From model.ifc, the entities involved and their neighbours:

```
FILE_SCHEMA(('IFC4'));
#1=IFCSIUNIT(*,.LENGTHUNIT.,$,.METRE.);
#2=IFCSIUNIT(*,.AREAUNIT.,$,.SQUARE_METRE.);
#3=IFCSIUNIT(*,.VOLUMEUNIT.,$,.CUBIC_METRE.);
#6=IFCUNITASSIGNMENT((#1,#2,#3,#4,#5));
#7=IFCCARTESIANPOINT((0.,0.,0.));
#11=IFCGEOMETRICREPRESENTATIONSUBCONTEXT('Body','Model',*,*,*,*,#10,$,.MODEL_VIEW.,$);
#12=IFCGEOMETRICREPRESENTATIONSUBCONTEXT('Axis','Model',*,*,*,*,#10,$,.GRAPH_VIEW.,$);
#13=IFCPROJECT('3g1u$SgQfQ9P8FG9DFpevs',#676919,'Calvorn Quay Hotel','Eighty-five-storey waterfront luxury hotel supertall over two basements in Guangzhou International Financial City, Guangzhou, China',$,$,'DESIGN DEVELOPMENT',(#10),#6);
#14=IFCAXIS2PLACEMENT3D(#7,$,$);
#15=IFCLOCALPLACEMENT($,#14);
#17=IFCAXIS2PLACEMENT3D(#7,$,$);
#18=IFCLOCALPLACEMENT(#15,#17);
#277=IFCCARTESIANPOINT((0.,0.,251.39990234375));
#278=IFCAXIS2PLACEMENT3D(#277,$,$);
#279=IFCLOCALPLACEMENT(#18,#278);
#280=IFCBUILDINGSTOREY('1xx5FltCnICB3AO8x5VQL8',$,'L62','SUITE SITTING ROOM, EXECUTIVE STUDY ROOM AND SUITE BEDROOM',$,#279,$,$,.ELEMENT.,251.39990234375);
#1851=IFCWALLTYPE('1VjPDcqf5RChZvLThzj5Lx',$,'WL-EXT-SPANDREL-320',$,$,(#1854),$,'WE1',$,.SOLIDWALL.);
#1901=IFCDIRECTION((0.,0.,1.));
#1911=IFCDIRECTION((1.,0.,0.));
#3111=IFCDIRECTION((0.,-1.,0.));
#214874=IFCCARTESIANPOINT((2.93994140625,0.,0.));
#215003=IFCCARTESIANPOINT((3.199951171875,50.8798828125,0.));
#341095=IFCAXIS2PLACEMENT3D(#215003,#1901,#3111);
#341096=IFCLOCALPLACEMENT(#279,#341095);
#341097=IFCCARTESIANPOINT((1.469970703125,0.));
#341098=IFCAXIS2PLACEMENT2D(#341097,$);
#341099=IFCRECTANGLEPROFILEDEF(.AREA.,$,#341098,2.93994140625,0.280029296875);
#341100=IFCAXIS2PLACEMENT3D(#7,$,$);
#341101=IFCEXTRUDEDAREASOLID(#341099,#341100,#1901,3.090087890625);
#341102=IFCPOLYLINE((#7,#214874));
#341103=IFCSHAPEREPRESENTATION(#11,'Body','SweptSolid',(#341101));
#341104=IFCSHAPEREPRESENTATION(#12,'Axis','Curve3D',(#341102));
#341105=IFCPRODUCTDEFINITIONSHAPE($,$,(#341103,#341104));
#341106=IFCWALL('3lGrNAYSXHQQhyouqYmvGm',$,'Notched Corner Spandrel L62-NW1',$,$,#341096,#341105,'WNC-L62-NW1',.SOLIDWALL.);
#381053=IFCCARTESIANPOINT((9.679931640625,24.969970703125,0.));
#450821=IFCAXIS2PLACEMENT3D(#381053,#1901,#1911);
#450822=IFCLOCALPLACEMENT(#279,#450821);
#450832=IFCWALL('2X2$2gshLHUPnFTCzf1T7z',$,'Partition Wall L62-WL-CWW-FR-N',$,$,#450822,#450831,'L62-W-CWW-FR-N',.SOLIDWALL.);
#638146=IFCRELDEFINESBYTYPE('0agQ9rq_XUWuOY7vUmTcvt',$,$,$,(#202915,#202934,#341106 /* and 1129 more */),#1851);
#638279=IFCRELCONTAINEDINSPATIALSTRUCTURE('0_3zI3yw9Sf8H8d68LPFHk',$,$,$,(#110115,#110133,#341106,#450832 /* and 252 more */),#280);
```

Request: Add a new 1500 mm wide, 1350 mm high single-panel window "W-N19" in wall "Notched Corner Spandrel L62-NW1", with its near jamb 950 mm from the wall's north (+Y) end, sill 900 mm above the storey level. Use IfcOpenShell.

```python
import numpy as np
import ifcopenshell
import ifcopenshell.api.feature
import ifcopenshell.api.geometry
import ifcopenshell.api.root
import ifcopenshell.api.spatial
import ifcopenshell.geom
import ifcopenshell.util.element
import ifcopenshell.util.placement
import ifcopenshell.util.representation
import ifcopenshell.util.shape
import ifcopenshell.util.unit

model = ifcopenshell.open("model.ifc")
unit_scale = ifcopenshell.util.unit.calculate_unit_scale(model)
settings = ifcopenshell.geom.settings()


def volume(element):
    """Net volume in cubic metres, openings subtracted."""
    shape = ifcopenshell.geom.create_shape(settings, element)
    return ifcopenshell.util.shape.get_volume(shape.geometry)


wall = model.by_guid("3lGrNAYSXHQQhyouqYmvGm")
storey = ifcopenshell.util.element.get_container(wall, ifc_class="IfcBuildingStorey")
context = ifcopenshell.util.representation.get_context(model, "Model", "Body", "MODEL_VIEW")
before = volume(wall)

width, height, from_end, sill = 1.5, 1.35, 0.95, 0.9  # metres

# The wall runs along its own X axis, and the end named is its -X end.
wall_shape = ifcopenshell.geom.create_shape(settings, wall)
x, y, z = ifcopenshell.util.shape.get_vertices(wall_shape.geometry).T
start = x.min() + from_end
face, thickness = float(y.min()), float(y.max() - y.min())
wall_matrix = ifcopenshell.util.placement.get_local_placement(wall.ObjectPlacement)
level = ifcopenshell.util.placement.get_local_placement(storey.ObjectPlacement)[2, 3]


def in_wall(x, y):
    """Placement at x, y metres in the wall's axes, at sill height."""
    matrix = wall_matrix.copy()
    matrix[:, 3] = wall_matrix @ np.array([x / unit_scale, y / unit_scale, 0.0, 1.0])
    matrix[2, 3] = level + sill / unit_scale
    return matrix


# Opening: a box that overshoots both wall faces by 50 mm.
opening = ifcopenshell.api.root.create_entity(model, ifc_class="IfcOpeningElement", predefined_type="OPENING")
box = ifcopenshell.api.geometry.add_wall_representation(
    model, context=context, length=width, height=height, thickness=thickness + 0.1
)
ifcopenshell.api.geometry.assign_representation(model, product=opening, representation=box)
ifcopenshell.api.geometry.edit_object_placement(model, product=opening, matrix=in_wall(start, face - 0.05), is_si=False)
ifcopenshell.api.feature.add_feature(model, feature=opening, element=wall)

window = ifcopenshell.api.root.create_entity(model, ifc_class="IfcWindow", name="W-N19", predefined_type="WINDOW")
window.OverallWidth, window.OverallHeight = width / unit_scale, height / unit_scale
window.PartitioningType = "SINGLE_PANEL"
body = ifcopenshell.api.geometry.add_window_representation(
    model,
    context=context,
    overall_width=window.OverallWidth,
    overall_height=window.OverallHeight,
    partition_type="SINGLE_PANEL",
)
ifcopenshell.api.geometry.assign_representation(model, product=window, representation=body)
ifcopenshell.api.spatial.assign_container(model, products=[window], relating_structure=storey)
ifcopenshell.api.feature.add_filling(model, opening=opening, element=window)

# Centre the window in the wall's thickness.
ifcopenshell.api.geometry.edit_object_placement(model, product=window, matrix=in_wall(start, face), is_si=False)
window_shape = ifcopenshell.geom.create_shape(settings, window)
depth = ifcopenshell.util.shape.get_vertices(window_shape.geometry)[:, 1]
offset = face + thickness / 2 - (depth.min() + depth.max()) / 2
ifcopenshell.api.geometry.edit_object_placement(model, product=window, matrix=in_wall(start, offset), is_si=False)

after = volume(wall)

print(f"wall volume {before:.3f} -> {after:.3f} m3")

model.write("model_v2.ifc")
```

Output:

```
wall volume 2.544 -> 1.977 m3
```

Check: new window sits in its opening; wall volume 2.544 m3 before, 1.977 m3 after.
